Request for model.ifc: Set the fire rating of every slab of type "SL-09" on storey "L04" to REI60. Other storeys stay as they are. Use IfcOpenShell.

First a look at what the model holds.

```python
import ifcopenshell
import ifcopenshell.util.element

model = ifcopenshell.open("model.ifc")
print(model.schema)
storey = next(s for s in model.by_type("IfcBuildingStorey") if s.Name == "L04")
slabs = [e for e in ifcopenshell.util.element.get_decomposition(storey) if e.is_a("IfcSlab")]
seen = {}
for e in slabs:
    element_type = ifcopenshell.util.element.get_type(e)
    key = (element_type.Name if element_type != e and element_type else None, ifcopenshell.util.element.get_pset(e, "Pset_SlabCommon", "FireRating"))
    seen[key] = seen.get(key, 0) + 1
for (name, value), count in sorted(seen.items(), key=str):
    print(count, "x", name, "|", value)
```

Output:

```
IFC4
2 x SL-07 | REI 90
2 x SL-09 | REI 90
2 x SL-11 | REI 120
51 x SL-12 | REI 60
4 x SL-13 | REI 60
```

```python
import ifcopenshell
import ifcopenshell.api.pset
import ifcopenshell.util.element

model = ifcopenshell.open("model.ifc")

storey = next(s for s in model.by_type("IfcBuildingStorey") if s.Name == "L04")
slabs = [e for e in ifcopenshell.util.element.get_decomposition(storey) if e.is_a("IfcSlab")]

count = 0
for e in slabs:
    element_type = ifcopenshell.util.element.get_type(e)
    if element_type in (None, e) or element_type.Name != "SL-09":
        continue
    # add_pset returns the element's existing set when there is one.
    pset = ifcopenshell.api.pset.add_pset(model, product=e, name="Pset_SlabCommon")
    ifcopenshell.api.pset.edit_pset(model, pset=pset, properties={"FireRating": "REI60"})
    count += 1

print(count, "slabs updated")

model.write("model-out.ifc")
```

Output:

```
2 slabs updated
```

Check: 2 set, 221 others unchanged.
